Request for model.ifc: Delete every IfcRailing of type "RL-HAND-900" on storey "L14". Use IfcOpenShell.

First a look at what the model holds.

```python
import ifcopenshell
import ifcopenshell.util.element

model = ifcopenshell.open("model.ifc")
print(model.schema)
storey = next(s for s in model.by_type("IfcBuildingStorey") if s.Name == "L14")
railings = [e for e in ifcopenshell.util.element.get_decomposition(storey) if e.is_a("IfcRailing")]
seen = {}
for e in railings:
    element_type = ifcopenshell.util.element.get_type(e)
    name = element_type.Name if element_type not in (None, e) else None
    seen[name] = seen.get(name, 0) + 1
for name, count in sorted(seen.items(), key=str):
    print(count, "x", name)
```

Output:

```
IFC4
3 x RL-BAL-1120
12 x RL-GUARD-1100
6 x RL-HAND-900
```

```python
import ifcopenshell
import ifcopenshell.api.root
import ifcopenshell.util.element

model = ifcopenshell.open("model.ifc")

storey = next(s for s in model.by_type("IfcBuildingStorey") if s.Name == "L14")
railings = [e for e in ifcopenshell.util.element.get_decomposition(storey) if e.is_a("IfcRailing")]
targets = [e for e in railings if (t := ifcopenshell.util.element.get_type(e)) not in (None, e) and t.Name == "RL-HAND-900"]

for e in targets:
    ifcopenshell.api.root.remove_product(model, product=e)
print(len(targets), "removed")

model.write("model_edited.ifc")
```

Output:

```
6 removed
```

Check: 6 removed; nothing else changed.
